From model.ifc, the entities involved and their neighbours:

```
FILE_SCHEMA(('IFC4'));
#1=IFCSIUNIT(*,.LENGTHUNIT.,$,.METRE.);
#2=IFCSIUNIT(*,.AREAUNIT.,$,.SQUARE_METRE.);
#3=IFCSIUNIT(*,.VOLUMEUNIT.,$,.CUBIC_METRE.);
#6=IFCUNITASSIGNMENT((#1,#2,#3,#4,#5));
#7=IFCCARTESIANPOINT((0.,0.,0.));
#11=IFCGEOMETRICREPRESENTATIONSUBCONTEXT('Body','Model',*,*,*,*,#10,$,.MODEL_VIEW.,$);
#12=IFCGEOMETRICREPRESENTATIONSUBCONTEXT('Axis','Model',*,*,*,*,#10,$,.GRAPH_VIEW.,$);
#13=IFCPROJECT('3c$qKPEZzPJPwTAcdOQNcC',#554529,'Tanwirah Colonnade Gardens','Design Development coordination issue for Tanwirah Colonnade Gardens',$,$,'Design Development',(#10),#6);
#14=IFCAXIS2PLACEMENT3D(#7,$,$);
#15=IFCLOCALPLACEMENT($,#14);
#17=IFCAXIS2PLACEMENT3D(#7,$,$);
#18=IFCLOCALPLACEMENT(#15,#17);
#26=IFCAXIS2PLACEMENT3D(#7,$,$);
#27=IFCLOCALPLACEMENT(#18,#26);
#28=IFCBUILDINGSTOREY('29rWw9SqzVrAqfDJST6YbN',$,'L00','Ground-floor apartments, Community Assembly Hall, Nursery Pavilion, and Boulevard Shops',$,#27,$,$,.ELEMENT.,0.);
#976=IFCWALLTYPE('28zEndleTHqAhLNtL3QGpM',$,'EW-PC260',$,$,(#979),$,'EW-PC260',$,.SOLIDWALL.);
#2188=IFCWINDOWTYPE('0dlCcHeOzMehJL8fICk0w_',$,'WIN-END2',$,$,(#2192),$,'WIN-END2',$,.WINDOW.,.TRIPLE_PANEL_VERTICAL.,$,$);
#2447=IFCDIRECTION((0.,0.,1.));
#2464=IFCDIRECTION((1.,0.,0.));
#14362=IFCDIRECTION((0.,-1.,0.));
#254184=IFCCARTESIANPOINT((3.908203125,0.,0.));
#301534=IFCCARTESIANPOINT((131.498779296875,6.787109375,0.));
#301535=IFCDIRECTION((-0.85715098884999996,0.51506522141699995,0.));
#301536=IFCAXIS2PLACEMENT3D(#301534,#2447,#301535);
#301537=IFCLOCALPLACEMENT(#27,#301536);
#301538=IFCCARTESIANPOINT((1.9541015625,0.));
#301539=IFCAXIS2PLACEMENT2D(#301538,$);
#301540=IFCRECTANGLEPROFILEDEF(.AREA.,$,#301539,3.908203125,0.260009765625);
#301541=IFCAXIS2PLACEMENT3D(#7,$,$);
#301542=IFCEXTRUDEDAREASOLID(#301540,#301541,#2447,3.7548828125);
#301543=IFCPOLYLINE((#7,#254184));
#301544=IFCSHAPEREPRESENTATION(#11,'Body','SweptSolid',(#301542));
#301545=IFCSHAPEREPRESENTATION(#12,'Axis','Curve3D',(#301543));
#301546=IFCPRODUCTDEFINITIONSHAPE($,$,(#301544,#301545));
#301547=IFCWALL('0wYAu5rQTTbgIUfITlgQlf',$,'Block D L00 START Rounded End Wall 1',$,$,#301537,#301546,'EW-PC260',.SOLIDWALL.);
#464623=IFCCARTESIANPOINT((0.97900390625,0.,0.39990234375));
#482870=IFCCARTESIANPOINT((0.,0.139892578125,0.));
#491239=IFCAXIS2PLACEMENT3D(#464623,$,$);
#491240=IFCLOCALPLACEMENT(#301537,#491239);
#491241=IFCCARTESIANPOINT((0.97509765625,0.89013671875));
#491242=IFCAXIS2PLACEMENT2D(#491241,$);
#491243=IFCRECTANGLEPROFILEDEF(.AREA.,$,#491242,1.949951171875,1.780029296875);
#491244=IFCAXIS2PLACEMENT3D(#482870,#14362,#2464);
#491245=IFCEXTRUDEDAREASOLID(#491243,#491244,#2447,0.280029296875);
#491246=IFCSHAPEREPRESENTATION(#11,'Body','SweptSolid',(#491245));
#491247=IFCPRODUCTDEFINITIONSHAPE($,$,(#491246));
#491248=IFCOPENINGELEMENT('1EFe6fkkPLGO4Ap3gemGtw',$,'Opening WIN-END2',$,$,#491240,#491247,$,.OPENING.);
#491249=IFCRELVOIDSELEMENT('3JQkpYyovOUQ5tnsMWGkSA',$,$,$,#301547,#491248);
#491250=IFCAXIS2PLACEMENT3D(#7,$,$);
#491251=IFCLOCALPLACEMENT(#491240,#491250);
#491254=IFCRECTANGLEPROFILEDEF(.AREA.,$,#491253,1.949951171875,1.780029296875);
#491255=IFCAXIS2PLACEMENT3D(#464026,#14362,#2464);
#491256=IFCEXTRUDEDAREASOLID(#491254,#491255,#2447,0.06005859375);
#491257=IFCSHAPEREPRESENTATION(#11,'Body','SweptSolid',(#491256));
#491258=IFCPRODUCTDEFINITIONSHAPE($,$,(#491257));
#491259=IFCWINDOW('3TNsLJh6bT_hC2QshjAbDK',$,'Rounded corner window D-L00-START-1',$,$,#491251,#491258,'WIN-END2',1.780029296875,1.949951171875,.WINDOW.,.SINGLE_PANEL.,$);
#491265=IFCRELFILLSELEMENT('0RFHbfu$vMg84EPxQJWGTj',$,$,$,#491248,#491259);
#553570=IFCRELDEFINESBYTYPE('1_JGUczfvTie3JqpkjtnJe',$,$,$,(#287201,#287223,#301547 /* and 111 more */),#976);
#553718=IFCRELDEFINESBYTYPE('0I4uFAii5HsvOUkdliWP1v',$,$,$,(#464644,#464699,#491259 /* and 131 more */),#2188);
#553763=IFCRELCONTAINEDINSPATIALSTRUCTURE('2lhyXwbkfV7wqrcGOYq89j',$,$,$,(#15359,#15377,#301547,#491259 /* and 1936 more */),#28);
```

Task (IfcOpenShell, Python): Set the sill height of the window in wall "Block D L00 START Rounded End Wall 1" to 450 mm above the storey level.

```python
import numpy as np
import ifcopenshell
import ifcopenshell.api.geometry
import ifcopenshell.geom
import ifcopenshell.util.element
import ifcopenshell.util.placement
import ifcopenshell.util.shape
import ifcopenshell.util.unit

model = ifcopenshell.open("model.ifc")
unit_scale = ifcopenshell.util.unit.calculate_unit_scale(model)

window = model.by_guid("3TNsLJh6bT_hC2QshjAbDK")
opening = window.FillsVoids[0].RelatingOpeningElement
storey = ifcopenshell.util.element.get_container(window, ifc_class="IfcBuildingStorey")
level = ifcopenshell.util.placement.get_local_placement(storey.ObjectPlacement)[2, 3]

# The opening's origin need not be at the sill, so measure its lowest point.
shape = ifcopenshell.geom.create_shape(ifcopenshell.geom.settings(), opening)
bottom = ifcopenshell.util.shape.get_shape_bottom_elevation(shape, shape.geometry) / unit_scale
dz = level + 0.45 / unit_scale - bottom

shift = np.array([0.0, 0.0, dz])
# The window is placed relative to its opening, so it follows when the opening moves.
matrix = ifcopenshell.util.placement.get_local_placement(opening.ObjectPlacement)
matrix[:3, 3] += shift
ifcopenshell.api.geometry.edit_object_placement(
    model, product=opening, matrix=matrix, is_si=False, should_transform_children=True
)

print(f"moved by {dz * unit_scale:+.3f} m")

model.write("model_rev.ifc")
```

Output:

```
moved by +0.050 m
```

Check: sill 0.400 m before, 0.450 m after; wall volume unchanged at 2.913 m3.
